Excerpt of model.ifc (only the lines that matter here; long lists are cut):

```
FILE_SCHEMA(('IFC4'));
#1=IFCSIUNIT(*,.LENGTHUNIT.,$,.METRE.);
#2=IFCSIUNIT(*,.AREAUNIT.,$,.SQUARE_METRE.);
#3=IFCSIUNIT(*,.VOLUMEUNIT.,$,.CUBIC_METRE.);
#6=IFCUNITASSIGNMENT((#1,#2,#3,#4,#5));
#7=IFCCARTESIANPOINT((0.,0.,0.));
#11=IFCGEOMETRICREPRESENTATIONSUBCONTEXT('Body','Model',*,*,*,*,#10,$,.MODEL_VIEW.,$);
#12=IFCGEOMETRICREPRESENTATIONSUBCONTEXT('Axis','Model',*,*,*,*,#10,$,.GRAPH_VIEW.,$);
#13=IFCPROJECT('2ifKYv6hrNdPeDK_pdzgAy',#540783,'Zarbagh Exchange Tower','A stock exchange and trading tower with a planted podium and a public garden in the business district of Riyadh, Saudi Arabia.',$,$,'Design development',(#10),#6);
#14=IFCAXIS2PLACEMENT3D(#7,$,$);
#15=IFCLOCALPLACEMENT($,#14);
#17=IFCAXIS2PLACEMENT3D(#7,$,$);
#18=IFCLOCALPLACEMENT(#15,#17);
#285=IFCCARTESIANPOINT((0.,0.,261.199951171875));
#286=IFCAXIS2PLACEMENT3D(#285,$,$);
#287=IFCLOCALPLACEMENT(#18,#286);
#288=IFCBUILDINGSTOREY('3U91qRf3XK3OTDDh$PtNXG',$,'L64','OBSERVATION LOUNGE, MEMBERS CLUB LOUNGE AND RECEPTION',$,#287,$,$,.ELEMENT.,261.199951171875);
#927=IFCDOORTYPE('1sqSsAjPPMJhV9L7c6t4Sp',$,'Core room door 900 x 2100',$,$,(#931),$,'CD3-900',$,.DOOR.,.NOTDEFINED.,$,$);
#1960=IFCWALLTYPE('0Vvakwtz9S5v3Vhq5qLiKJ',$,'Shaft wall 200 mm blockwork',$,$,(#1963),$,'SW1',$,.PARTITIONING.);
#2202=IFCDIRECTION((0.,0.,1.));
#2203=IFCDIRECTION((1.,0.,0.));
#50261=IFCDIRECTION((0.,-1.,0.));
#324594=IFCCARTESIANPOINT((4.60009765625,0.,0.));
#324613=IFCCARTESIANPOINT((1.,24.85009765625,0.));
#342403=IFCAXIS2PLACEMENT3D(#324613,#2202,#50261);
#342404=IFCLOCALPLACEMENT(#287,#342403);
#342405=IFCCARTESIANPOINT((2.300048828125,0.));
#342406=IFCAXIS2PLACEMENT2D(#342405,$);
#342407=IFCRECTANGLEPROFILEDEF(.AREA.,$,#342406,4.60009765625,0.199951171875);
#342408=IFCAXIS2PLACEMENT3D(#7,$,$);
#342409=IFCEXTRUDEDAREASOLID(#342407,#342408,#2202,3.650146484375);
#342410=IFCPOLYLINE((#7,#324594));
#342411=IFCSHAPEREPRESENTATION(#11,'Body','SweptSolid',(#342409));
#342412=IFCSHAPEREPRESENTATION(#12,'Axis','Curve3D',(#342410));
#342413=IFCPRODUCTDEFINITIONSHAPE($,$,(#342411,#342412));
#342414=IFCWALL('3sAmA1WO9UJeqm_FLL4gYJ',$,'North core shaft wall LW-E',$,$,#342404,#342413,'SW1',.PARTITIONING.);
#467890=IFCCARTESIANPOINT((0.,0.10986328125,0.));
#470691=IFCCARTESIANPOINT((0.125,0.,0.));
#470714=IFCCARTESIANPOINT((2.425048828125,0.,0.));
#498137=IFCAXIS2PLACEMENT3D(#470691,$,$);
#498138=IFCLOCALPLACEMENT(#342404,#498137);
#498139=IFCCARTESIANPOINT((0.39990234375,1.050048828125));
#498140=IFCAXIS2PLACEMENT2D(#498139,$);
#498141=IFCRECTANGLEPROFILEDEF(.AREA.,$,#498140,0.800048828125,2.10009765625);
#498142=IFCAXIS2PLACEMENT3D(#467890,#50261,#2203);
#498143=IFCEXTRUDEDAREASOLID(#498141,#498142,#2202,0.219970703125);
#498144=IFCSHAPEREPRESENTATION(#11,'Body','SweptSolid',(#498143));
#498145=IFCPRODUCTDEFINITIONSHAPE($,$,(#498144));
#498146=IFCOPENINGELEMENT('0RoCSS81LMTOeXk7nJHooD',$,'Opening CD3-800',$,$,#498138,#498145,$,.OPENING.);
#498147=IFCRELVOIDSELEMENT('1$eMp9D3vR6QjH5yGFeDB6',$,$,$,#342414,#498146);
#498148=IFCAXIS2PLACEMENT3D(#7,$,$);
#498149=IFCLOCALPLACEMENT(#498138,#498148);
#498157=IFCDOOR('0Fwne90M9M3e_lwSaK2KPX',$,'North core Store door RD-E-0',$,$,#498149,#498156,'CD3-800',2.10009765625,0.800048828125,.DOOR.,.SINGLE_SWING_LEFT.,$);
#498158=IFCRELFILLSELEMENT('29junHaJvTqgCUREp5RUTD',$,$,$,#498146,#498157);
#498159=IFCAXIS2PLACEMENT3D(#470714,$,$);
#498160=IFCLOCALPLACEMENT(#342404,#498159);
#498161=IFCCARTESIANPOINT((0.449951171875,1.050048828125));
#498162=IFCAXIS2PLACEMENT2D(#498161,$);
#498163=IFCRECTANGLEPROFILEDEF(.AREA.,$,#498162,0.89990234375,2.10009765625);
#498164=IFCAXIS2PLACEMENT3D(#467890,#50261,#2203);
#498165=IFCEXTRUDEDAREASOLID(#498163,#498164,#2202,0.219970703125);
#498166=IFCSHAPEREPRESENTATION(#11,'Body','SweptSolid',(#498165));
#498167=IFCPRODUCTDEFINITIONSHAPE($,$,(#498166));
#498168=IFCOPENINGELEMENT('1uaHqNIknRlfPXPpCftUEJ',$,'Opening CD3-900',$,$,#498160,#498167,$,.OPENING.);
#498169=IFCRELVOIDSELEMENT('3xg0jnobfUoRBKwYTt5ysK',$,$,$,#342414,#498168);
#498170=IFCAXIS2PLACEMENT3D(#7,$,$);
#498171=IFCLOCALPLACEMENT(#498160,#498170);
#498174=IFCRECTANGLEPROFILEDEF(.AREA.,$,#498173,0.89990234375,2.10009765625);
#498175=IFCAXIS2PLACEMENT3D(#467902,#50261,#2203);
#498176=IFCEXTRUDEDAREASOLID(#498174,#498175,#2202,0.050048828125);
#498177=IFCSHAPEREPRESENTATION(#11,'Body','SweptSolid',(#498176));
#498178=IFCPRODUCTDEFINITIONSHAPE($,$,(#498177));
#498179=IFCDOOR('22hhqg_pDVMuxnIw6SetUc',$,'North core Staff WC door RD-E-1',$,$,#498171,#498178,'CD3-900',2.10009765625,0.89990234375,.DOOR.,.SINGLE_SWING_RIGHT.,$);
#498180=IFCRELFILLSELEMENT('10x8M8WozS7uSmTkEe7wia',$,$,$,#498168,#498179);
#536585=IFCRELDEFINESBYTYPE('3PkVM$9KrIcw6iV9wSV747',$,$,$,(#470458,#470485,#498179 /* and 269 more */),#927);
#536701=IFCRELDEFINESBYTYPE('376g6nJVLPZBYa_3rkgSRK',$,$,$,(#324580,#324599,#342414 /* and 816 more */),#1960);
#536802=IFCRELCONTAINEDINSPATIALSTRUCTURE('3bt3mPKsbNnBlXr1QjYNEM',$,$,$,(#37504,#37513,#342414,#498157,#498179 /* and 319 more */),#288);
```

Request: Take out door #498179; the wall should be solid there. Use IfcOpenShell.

```python
import ifcopenshell
import ifcopenshell.api.feature
import ifcopenshell.api.root
import ifcopenshell.geom
import ifcopenshell.util.shape

model = ifcopenshell.open("model.ifc")
settings = ifcopenshell.geom.settings()


def volume(element):
    """Net volume in cubic metres, openings subtracted."""
    shape = ifcopenshell.geom.create_shape(settings, element)
    return ifcopenshell.util.shape.get_volume(shape.geometry)


door = model.by_guid("22hhqg_pDVMuxnIw6SetUc")
opening = door.FillsVoids[0].RelatingOpeningElement
wall = opening.VoidsElements[0].RelatingBuildingElement
before = volume(wall)

ifcopenshell.api.root.remove_product(model, product=door)
ifcopenshell.api.feature.remove_feature(model, feature=opening)

after = volume(wall)

print(f"wall volume {before:.3f} -> {after:.3f} m3")

model.write("model_edited.ifc")
```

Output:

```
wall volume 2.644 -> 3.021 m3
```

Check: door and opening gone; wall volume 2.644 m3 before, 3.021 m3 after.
